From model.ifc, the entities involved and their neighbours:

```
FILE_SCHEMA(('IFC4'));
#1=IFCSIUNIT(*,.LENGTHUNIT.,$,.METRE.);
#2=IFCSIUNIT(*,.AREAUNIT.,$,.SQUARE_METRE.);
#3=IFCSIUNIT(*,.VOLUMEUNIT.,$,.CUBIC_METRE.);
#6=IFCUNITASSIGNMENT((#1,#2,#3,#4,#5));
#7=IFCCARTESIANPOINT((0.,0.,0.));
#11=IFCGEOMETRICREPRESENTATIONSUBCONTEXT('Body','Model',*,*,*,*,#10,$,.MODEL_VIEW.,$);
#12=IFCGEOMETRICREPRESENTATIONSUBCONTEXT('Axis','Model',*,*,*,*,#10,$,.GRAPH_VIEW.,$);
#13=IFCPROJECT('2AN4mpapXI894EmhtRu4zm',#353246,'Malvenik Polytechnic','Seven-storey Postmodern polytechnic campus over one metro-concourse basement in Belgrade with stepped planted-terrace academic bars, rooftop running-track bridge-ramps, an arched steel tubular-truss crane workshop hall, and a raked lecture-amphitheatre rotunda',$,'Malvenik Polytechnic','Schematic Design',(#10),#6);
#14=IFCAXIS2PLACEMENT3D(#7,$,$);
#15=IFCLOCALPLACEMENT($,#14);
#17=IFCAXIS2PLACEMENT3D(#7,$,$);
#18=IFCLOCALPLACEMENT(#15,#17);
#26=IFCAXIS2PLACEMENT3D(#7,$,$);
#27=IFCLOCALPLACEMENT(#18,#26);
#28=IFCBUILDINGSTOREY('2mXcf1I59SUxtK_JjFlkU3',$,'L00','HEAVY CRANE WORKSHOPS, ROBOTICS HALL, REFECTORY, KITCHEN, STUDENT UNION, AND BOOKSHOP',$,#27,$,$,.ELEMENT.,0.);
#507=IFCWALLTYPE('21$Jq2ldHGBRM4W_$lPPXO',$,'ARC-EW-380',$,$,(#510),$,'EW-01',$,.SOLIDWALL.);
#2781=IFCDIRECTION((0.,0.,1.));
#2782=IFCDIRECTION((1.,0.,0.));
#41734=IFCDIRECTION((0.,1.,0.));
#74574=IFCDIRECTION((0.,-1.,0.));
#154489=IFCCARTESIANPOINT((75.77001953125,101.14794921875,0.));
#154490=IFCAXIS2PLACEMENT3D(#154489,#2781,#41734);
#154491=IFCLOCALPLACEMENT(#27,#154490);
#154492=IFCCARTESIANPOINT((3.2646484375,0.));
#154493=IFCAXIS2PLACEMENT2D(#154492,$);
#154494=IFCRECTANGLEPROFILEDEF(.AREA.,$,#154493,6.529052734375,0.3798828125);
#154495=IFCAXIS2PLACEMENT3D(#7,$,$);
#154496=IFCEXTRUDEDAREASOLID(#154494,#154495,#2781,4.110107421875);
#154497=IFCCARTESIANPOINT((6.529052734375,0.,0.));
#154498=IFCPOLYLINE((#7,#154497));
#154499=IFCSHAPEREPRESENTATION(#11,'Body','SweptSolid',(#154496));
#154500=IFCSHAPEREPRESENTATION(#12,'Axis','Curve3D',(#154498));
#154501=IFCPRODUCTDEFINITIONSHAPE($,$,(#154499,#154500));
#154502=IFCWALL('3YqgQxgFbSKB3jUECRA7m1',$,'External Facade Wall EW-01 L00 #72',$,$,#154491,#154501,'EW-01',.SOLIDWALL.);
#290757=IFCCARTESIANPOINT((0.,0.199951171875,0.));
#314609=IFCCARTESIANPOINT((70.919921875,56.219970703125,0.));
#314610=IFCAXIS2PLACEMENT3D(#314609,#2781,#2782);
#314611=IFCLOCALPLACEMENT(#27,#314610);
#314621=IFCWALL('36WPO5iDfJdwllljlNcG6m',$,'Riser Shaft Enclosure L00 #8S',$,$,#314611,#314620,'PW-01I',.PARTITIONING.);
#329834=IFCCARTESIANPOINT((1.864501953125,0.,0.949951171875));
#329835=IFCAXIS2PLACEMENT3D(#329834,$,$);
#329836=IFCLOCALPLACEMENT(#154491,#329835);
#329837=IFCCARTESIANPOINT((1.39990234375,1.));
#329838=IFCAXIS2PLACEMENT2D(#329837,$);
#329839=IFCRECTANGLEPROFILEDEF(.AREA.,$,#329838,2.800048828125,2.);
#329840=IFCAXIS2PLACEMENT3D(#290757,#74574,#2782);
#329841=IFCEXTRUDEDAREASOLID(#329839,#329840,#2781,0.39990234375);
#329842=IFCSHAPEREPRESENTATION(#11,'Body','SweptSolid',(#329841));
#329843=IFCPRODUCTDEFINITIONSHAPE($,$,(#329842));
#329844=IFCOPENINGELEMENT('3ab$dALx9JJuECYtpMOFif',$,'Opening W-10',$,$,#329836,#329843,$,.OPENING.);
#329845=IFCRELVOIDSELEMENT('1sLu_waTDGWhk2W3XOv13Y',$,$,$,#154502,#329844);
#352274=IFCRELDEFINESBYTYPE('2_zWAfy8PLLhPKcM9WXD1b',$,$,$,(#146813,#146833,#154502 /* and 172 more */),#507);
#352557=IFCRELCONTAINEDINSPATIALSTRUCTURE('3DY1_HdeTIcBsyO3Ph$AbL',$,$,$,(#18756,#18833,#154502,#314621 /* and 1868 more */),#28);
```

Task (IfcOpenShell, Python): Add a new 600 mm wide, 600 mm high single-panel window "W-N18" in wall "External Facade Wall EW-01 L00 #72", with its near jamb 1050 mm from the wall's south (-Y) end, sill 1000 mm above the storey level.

```python
import numpy as np
import ifcopenshell
import ifcopenshell.api.feature
import ifcopenshell.api.geometry
import ifcopenshell.api.root
import ifcopenshell.api.spatial
import ifcopenshell.geom
import ifcopenshell.util.element
import ifcopenshell.util.placement
import ifcopenshell.util.representation
import ifcopenshell.util.shape
import ifcopenshell.util.unit

model = ifcopenshell.open("model.ifc")
unit_scale = ifcopenshell.util.unit.calculate_unit_scale(model)
settings = ifcopenshell.geom.settings()


def volume(element):
    """Net volume in cubic metres, openings subtracted."""
    shape = ifcopenshell.geom.create_shape(settings, element)
    return ifcopenshell.util.shape.get_volume(shape.geometry)


wall = model.by_id(154502)
storey = ifcopenshell.util.element.get_container(wall, ifc_class="IfcBuildingStorey")
context = ifcopenshell.util.representation.get_context(model, "Model", "Body", "MODEL_VIEW")
before = volume(wall)

width, height, from_end, sill = 0.6, 0.6, 1.05, 1  # metres

# The wall runs along its own X axis, and the end named is its -X end.
wall_shape = ifcopenshell.geom.create_shape(settings, wall)
x, y, z = ifcopenshell.util.shape.get_vertices(wall_shape.geometry).T
start = x.min() + from_end
face, thickness = float(y.min()), float(y.max() - y.min())
wall_matrix = ifcopenshell.util.placement.get_local_placement(wall.ObjectPlacement)
level = ifcopenshell.util.placement.get_local_placement(storey.ObjectPlacement)[2, 3]


def in_wall(x, y):
    """Placement at x, y metres in the wall's axes, at sill height."""
    matrix = wall_matrix.copy()
    matrix[:, 3] = wall_matrix @ np.array([x / unit_scale, y / unit_scale, 0.0, 1.0])
    matrix[2, 3] = level + sill / unit_scale
    return matrix


# Opening: a box that overshoots both wall faces by 50 mm.
opening = ifcopenshell.api.root.create_entity(model, ifc_class="IfcOpeningElement", predefined_type="OPENING")
box = ifcopenshell.api.geometry.add_wall_representation(
    model, context=context, length=width, height=height, thickness=thickness + 0.1
)
ifcopenshell.api.geometry.assign_representation(model, product=opening, representation=box)
ifcopenshell.api.geometry.edit_object_placement(model, product=opening, matrix=in_wall(start, face - 0.05), is_si=False)
ifcopenshell.api.feature.add_feature(model, feature=opening, element=wall)

window = ifcopenshell.api.root.create_entity(model, ifc_class="IfcWindow", name="W-N18", predefined_type="WINDOW")
window.OverallWidth, window.OverallHeight = width / unit_scale, height / unit_scale
window.PartitioningType = "SINGLE_PANEL"
body = ifcopenshell.api.geometry.add_window_representation(
    model,
    context=context,
    overall_width=window.OverallWidth,
    overall_height=window.OverallHeight,
    partition_type="SINGLE_PANEL",
)
ifcopenshell.api.geometry.assign_representation(model, product=window, representation=body)
ifcopenshell.api.spatial.assign_container(model, products=[window], relating_structure=storey)
ifcopenshell.api.feature.add_filling(model, opening=opening, element=window)

# Centre the window in the wall's thickness.
ifcopenshell.api.geometry.edit_object_placement(model, product=window, matrix=in_wall(start, face), is_si=False)
window_shape = ifcopenshell.geom.create_shape(settings, window)
depth = ifcopenshell.util.shape.get_vertices(window_shape.geometry)[:, 1]
offset = face + thickness / 2 - (depth.min() + depth.max()) / 2
ifcopenshell.api.geometry.edit_object_placement(model, product=window, matrix=in_wall(start, offset), is_si=False)

after = volume(wall)

print(f"wall volume {before:.3f} -> {after:.3f} m3")

model.write("model_v2.ifc")
```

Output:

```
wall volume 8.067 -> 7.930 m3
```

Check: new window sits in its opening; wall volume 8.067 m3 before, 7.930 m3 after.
